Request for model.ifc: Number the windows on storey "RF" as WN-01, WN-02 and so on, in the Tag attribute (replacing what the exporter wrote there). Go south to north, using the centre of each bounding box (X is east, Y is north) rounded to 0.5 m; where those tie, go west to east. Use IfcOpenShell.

First a look at what the model holds.

```python
import ifcopenshell
import ifcopenshell.util.element
import ifcopenshell.util.placement

model = ifcopenshell.open("model.ifc")
print(model.schema)
storey = next(s for s in model.by_type("IfcBuildingStorey") if s.Name == "RF")
windows = [e for e in ifcopenshell.util.element.get_decomposition(storey) if e.is_a("IfcWindow")]
for e in sorted(windows, key=lambda e: e.id()):
    origin = ifcopenshell.util.placement.get_local_placement(e.ObjectPlacement)[:3, 3]
    print(e.id(), e.Tag, e.Name, origin.round(2) + 0.0, sep=" | ")
```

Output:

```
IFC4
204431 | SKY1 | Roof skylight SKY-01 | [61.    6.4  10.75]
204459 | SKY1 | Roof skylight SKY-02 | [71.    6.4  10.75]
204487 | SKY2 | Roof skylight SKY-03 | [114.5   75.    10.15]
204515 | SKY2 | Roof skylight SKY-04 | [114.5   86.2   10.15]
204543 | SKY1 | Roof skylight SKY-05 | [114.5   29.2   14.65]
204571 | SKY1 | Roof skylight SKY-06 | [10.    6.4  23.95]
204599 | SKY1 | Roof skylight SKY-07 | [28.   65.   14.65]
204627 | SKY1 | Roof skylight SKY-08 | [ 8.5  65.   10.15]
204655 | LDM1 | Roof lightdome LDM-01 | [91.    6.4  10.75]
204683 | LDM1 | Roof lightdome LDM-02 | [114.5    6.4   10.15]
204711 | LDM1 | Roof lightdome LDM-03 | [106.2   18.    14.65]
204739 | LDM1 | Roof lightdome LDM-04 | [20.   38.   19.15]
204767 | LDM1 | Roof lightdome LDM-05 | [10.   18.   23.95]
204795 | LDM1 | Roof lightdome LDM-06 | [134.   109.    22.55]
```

```python
import ifcopenshell
import ifcopenshell.geom
import ifcopenshell.util.element
import ifcopenshell.util.shape

model = ifcopenshell.open("model.ifc")
settings = ifcopenshell.geom.settings()
settings.set("use-world-coords", True)


def centre(element):
    shape = ifcopenshell.geom.create_shape(settings, element)
    return ifcopenshell.util.shape.get_bbox_centroid(shape.geometry)


storey = next(s for s in model.by_type("IfcBuildingStorey") if s.Name == "RF")
windows = [e for e in ifcopenshell.util.element.get_decomposition(storey) if e.is_a("IfcWindow")]

# Insertion points can sit at a corner or the storey origin, so sort by the geometry (in metres).
centres = {e: centre(e) for e in windows}
windows.sort(key=lambda e: (round(centres[e][1] / 0.5), centres[e][0]))

for i, e in enumerate(windows, start=1):
    number = f"WN-{i:02d}"
    e.Tag = number
    print(e.id(), number)

model.write("model_edited.ifc")
```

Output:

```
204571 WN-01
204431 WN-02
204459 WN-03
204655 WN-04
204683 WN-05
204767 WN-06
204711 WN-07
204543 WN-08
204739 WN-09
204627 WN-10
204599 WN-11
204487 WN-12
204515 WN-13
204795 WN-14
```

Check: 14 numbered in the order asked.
